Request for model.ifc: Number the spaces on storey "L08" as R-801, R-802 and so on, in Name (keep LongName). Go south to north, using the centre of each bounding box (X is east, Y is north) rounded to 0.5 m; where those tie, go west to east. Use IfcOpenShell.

First a look at what the model holds.

```python
import ifcopenshell
import ifcopenshell.util.element
import ifcopenshell.util.placement

model = ifcopenshell.open("model.ifc")
print(model.schema)
storey = next(s for s in model.by_type("IfcBuildingStorey") if s.Name == "L08")
spaces = [e for e in ifcopenshell.util.element.get_decomposition(storey) if e.is_a("IfcSpace")]
for e in sorted(spaces, key=lambda e: e.id()):
    origin = ifcopenshell.util.placement.get_local_placement(e.ObjectPlacement)[:3, 3]
    print(e.id(), e.Name, e.LongName, origin.round(2) + 0.0, sep=" | ")
```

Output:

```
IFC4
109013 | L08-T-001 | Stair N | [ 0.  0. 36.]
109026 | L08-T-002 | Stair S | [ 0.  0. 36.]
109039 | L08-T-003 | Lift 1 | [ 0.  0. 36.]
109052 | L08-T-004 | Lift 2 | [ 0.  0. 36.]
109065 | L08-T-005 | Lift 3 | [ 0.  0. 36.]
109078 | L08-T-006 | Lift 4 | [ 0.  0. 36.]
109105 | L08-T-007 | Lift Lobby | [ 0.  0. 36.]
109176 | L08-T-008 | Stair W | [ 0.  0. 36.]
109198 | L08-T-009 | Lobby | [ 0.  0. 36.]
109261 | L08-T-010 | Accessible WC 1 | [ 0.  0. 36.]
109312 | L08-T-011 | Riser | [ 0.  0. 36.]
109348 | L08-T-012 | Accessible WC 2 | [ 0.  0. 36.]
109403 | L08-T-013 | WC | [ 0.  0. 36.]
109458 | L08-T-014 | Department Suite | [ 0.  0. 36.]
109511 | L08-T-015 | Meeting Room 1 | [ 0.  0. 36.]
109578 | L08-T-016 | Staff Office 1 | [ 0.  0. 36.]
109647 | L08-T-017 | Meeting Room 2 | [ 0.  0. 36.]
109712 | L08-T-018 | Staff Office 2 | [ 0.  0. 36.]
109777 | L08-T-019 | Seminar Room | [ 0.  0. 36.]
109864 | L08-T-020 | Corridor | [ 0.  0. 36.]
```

```python
import ifcopenshell
import ifcopenshell.geom
import ifcopenshell.util.element
import ifcopenshell.util.shape

model = ifcopenshell.open("model.ifc")
settings = ifcopenshell.geom.settings()
settings.set("use-world-coords", True)


def centre(element):
    shape = ifcopenshell.geom.create_shape(settings, element)
    return ifcopenshell.util.shape.get_bbox_centroid(shape.geometry)


storey = next(s for s in model.by_type("IfcBuildingStorey") if s.Name == "L08")
spaces = [e for e in ifcopenshell.util.element.get_decomposition(storey) if e.is_a("IfcSpace")]

# Insertion points can sit at a corner or the storey origin, so sort by the geometry (in metres).
centres = {e: centre(e) for e in spaces}
spaces.sort(key=lambda e: (round(centres[e][1] / 0.5), centres[e][0]))

for i, e in enumerate(spaces, start=1):
    number = f"R-8{i:02d}"
    e.Name = number
    print(e.id(), number)

model.write("model_rev.ifc")
```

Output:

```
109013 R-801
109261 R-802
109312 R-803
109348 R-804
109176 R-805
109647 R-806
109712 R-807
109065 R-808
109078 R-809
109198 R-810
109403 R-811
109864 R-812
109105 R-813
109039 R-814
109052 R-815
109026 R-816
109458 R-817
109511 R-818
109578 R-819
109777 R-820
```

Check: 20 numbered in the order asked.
